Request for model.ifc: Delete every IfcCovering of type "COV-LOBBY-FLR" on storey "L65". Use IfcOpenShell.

First a look at what the model holds.

```python
import ifcopenshell
import ifcopenshell.util.element

model = ifcopenshell.open("model.ifc")
print(model.schema)
storey = next(s for s in model.by_type("IfcBuildingStorey") if s.Name == "L65")
coverings = [e for e in ifcopenshell.util.element.get_decomposition(storey) if e.is_a("IfcCovering")]
seen = {}
for e in coverings:
    element_type = ifcopenshell.util.element.get_type(e)
    name = element_type.Name if element_type not in (None, e) else None
    seen[name] = seen.get(name, 0) + 1
for name, count in sorted(seen.items(), key=str):
    print(count, "x", name)
```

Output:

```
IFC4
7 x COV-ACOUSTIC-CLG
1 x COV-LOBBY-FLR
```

```python
import ifcopenshell
import ifcopenshell.api.root
import ifcopenshell.util.element

model = ifcopenshell.open("model.ifc")

storey = next(s for s in model.by_type("IfcBuildingStorey") if s.Name == "L65")
coverings = [e for e in ifcopenshell.util.element.get_decomposition(storey) if e.is_a("IfcCovering")]
targets = [e for e in coverings if (t := ifcopenshell.util.element.get_type(e)) not in (None, e) and t.Name == "COV-LOBBY-FLR"]

for e in targets:
    ifcopenshell.api.root.remove_product(model, product=e)
print(len(targets), "removed")

model.write("model_rev.ifc")
```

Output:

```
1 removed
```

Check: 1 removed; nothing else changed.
